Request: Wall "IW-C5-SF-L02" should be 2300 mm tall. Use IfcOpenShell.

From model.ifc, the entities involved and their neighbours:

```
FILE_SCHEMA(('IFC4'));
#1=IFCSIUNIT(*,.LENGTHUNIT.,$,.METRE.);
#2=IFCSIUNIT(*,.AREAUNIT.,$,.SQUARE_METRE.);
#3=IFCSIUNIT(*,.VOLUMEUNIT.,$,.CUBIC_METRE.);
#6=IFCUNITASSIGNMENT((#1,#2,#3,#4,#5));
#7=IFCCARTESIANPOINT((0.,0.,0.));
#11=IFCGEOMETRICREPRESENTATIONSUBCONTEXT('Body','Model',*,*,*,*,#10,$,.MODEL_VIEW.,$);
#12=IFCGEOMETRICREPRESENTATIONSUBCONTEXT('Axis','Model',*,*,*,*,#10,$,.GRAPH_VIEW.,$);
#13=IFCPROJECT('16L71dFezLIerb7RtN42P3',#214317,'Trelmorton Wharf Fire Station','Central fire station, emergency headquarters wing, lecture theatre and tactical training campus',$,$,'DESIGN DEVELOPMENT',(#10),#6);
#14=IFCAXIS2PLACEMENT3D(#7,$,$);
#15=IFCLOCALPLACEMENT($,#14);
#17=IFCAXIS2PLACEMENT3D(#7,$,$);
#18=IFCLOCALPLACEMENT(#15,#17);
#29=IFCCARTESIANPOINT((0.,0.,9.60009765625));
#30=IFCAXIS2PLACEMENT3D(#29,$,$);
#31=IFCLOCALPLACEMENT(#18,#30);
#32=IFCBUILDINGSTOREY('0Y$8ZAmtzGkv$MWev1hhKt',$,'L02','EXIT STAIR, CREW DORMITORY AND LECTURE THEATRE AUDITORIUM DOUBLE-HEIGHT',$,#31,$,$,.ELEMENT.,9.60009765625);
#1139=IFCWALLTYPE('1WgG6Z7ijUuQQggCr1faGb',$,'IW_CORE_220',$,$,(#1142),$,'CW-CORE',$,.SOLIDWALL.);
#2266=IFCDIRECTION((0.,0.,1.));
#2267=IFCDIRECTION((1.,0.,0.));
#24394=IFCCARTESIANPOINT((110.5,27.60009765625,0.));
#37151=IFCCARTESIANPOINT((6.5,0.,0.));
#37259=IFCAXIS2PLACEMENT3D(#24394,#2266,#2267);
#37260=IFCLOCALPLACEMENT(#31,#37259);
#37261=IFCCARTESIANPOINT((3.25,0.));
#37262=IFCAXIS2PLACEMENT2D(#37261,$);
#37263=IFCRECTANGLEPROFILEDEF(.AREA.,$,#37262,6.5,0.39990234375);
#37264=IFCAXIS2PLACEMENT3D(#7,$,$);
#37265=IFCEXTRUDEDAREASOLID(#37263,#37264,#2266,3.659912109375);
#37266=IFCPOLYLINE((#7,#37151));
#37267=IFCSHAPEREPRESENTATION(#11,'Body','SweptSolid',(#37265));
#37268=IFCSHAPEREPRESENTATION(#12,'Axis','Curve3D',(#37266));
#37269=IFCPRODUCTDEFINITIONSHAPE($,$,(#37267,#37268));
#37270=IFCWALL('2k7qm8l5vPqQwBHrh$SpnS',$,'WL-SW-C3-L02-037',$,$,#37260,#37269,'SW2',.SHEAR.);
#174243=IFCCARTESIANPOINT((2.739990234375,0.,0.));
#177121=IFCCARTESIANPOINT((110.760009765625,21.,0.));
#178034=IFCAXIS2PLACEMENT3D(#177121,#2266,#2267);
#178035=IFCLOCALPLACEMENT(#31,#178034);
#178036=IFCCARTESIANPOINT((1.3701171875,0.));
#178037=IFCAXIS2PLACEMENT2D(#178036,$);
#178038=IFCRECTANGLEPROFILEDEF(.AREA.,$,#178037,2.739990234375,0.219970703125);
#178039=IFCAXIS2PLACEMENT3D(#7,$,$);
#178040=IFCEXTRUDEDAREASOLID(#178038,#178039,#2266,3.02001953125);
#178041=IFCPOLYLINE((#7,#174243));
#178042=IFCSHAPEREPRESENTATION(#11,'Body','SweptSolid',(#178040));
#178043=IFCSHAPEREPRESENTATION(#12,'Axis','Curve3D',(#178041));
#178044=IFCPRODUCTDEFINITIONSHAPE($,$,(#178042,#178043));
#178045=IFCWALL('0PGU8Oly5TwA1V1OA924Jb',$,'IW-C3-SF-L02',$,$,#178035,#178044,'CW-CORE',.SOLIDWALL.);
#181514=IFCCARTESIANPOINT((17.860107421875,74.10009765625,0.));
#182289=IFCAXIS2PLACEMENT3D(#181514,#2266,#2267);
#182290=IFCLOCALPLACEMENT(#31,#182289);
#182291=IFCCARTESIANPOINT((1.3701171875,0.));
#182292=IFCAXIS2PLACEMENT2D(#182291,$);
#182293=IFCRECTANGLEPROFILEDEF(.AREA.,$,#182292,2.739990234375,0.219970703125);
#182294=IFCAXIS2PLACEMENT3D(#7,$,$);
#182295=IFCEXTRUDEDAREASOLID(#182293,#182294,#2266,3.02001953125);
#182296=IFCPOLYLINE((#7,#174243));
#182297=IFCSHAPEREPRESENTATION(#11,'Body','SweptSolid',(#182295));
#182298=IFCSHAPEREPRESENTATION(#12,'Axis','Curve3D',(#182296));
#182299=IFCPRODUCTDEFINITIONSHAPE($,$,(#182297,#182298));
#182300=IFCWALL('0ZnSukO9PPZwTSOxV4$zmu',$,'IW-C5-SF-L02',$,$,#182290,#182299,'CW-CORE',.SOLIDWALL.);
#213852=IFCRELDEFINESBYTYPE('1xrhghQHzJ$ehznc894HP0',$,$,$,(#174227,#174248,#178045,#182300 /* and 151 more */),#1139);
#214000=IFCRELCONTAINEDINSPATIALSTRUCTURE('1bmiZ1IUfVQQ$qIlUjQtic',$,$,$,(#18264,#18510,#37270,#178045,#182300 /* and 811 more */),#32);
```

```python
import ifcopenshell
import ifcopenshell.geom
import ifcopenshell.util.representation
import ifcopenshell.util.shape
import ifcopenshell.util.unit

model = ifcopenshell.open("model.ifc")
unit_scale = ifcopenshell.util.unit.calculate_unit_scale(model)
settings = ifcopenshell.geom.settings()


def volume(element):
    """Net volume in cubic metres, openings subtracted."""
    shape = ifcopenshell.geom.create_shape(settings, element)
    return ifcopenshell.util.shape.get_volume(shape.geometry)


wall = model.by_guid("0ZnSukO9PPZwTSOxV4$zmu")
before = volume(wall)

body = ifcopenshell.util.representation.get_representation(wall, "Model", "Body")
solid = body.Items[0]
old_height = solid.Depth
solid.Depth = 2.3 / unit_scale
after = volume(wall)

print(f"height {old_height:g} -> {solid.Depth:g}, volume {before:.3f} -> {after:.3f} m3")

model.write("model_updated.ifc")
```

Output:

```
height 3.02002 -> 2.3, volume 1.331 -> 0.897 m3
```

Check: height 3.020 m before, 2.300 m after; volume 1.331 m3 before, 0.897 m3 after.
